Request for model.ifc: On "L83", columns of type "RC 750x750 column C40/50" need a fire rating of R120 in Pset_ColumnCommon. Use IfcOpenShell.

First a look at what the model holds.

```python
import ifcopenshell
import ifcopenshell.util.element

model = ifcopenshell.open("model.ifc")
print(model.schema)
storey = next(s for s in model.by_type("IfcBuildingStorey") if s.Name == "L83")
columns = [e for e in ifcopenshell.util.element.get_decomposition(storey) if e.is_a("IfcColumn")]
seen = {}
for e in columns:
    element_type = ifcopenshell.util.element.get_type(e)
    key = (element_type.Name if element_type != e and element_type else None, ifcopenshell.util.element.get_pset(e, "Pset_ColumnCommon", "FireRating"))
    seen[key] = seen.get(key, 0) + 1
for (name, value), count in sorted(seen.items(), key=str):
    print(count, "x", name, "|", value)
```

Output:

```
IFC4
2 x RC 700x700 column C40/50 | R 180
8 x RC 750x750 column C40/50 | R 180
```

```python
import ifcopenshell
import ifcopenshell.api.pset
import ifcopenshell.util.element

model = ifcopenshell.open("model.ifc")

storey = next(s for s in model.by_type("IfcBuildingStorey") if s.Name == "L83")
columns = [e for e in ifcopenshell.util.element.get_decomposition(storey) if e.is_a("IfcColumn")]

count = 0
for e in columns:
    element_type = ifcopenshell.util.element.get_type(e)
    if element_type in (None, e) or element_type.Name != "RC 750x750 column C40/50":
        continue
    found = ifcopenshell.util.element.get_pset(e, "Pset_ColumnCommon", should_inherit=False)
    if found:
        pset = model.by_id(found["id"])
        if len(ifcopenshell.util.element.get_elements_by_pset(pset)) > 1:
            pset = ifcopenshell.api.pset.unshare_pset(model, products=[e], pset=pset)[0]
    else:
        pset = ifcopenshell.api.pset.add_pset(model, product=e, name="Pset_ColumnCommon")
    ifcopenshell.api.pset.edit_pset(model, pset=pset, properties={"FireRating": "R120"})
    count += 1

print(count, "columns updated")

model.write("model_updated.ifc")
```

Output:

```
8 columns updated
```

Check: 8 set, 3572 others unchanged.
